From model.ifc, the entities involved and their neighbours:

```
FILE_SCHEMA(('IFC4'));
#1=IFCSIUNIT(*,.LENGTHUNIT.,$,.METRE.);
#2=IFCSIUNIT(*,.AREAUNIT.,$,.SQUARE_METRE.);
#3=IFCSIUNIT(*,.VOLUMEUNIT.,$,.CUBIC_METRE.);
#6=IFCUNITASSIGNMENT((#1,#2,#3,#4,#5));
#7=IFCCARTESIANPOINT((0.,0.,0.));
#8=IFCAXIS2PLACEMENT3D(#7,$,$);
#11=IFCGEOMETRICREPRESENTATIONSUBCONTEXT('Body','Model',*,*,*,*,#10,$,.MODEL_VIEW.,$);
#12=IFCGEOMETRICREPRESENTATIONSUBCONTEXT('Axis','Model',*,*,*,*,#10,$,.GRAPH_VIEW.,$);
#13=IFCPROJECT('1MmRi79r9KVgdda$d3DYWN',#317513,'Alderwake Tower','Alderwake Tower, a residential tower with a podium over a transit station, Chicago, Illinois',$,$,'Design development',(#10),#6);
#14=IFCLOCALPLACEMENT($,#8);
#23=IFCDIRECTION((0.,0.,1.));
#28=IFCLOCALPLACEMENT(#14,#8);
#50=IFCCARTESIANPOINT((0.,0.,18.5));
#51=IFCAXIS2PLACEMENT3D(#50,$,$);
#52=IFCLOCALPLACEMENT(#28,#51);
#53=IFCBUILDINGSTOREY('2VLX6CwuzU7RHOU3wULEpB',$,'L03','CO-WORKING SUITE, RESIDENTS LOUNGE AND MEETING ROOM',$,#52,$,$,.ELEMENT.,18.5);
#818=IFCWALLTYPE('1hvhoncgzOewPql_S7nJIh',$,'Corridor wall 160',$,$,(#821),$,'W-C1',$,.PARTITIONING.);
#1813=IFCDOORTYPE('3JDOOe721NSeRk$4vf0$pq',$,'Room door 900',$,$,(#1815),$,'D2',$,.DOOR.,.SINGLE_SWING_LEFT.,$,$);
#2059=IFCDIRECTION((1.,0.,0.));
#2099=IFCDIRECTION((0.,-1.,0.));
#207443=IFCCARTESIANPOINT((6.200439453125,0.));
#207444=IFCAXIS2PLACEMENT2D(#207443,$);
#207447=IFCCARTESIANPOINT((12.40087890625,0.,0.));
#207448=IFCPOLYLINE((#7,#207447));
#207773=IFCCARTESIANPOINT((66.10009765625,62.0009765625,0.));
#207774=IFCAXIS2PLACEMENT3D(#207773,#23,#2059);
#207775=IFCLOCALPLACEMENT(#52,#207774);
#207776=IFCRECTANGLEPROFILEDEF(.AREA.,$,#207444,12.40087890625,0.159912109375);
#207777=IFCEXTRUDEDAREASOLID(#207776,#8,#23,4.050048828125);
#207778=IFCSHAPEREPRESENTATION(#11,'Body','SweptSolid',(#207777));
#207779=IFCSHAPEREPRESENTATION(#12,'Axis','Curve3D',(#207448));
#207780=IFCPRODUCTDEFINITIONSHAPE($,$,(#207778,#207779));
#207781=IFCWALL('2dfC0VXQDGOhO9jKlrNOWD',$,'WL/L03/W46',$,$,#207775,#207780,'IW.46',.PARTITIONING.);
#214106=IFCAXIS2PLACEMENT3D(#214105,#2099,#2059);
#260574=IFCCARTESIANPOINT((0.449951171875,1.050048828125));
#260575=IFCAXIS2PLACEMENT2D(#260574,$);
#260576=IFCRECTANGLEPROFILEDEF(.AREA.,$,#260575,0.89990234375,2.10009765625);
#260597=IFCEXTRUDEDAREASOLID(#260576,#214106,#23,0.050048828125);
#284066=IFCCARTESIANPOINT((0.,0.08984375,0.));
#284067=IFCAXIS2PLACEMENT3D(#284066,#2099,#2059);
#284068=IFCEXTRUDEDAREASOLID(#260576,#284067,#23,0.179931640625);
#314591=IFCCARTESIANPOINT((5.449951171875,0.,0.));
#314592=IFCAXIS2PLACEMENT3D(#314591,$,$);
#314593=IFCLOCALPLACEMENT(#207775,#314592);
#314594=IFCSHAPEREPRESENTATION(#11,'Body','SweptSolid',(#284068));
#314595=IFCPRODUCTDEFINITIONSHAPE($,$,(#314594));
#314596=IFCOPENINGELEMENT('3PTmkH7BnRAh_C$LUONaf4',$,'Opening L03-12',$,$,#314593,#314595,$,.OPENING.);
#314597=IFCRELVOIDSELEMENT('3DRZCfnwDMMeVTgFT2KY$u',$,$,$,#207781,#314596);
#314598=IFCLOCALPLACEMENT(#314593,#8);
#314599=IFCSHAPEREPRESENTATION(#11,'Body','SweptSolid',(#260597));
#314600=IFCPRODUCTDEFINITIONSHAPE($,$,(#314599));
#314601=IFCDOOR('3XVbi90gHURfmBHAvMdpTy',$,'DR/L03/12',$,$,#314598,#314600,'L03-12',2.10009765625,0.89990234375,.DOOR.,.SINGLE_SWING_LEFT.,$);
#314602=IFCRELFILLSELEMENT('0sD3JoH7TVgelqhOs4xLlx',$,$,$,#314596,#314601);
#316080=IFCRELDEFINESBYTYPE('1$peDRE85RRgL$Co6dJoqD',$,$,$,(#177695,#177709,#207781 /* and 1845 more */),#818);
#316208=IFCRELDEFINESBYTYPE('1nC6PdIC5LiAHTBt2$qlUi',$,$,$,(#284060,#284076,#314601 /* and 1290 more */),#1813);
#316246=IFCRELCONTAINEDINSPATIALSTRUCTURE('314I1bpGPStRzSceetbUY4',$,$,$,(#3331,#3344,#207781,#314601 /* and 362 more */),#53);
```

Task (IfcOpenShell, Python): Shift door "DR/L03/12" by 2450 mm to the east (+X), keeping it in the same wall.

```python
import ifcopenshell
import ifcopenshell.api.geometry
import ifcopenshell.util.placement
import ifcopenshell.util.unit

model = ifcopenshell.open("model.ifc")
unit_scale = ifcopenshell.util.unit.calculate_unit_scale(model)

door = model.by_guid("3XVbi90gHURfmBHAvMdpTy")
opening = door.FillsVoids[0].RelatingOpeningElement
wall = opening.VoidsElements[0].RelatingBuildingElement

wall_matrix = ifcopenshell.util.placement.get_local_placement(wall.ObjectPlacement)
shift = wall_matrix[:3, 0] * 2.45 / unit_scale
before = ifcopenshell.util.placement.get_local_placement(door.ObjectPlacement)[:3, 3].copy()

# The door is placed relative to its opening, so it follows when the opening moves.
matrix = ifcopenshell.util.placement.get_local_placement(opening.ObjectPlacement)
matrix[:3, 3] += shift
ifcopenshell.api.geometry.edit_object_placement(
    model, product=opening, matrix=matrix, is_si=False, should_transform_children=True
)

after = ifcopenshell.util.placement.get_local_placement(door.ObjectPlacement)[:3, 3]
print("door moved by", (after - before).round(3) + 0.0)

model.write("model_v2.ifc")
```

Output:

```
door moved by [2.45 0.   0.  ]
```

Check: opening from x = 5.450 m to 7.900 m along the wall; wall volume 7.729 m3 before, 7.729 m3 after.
